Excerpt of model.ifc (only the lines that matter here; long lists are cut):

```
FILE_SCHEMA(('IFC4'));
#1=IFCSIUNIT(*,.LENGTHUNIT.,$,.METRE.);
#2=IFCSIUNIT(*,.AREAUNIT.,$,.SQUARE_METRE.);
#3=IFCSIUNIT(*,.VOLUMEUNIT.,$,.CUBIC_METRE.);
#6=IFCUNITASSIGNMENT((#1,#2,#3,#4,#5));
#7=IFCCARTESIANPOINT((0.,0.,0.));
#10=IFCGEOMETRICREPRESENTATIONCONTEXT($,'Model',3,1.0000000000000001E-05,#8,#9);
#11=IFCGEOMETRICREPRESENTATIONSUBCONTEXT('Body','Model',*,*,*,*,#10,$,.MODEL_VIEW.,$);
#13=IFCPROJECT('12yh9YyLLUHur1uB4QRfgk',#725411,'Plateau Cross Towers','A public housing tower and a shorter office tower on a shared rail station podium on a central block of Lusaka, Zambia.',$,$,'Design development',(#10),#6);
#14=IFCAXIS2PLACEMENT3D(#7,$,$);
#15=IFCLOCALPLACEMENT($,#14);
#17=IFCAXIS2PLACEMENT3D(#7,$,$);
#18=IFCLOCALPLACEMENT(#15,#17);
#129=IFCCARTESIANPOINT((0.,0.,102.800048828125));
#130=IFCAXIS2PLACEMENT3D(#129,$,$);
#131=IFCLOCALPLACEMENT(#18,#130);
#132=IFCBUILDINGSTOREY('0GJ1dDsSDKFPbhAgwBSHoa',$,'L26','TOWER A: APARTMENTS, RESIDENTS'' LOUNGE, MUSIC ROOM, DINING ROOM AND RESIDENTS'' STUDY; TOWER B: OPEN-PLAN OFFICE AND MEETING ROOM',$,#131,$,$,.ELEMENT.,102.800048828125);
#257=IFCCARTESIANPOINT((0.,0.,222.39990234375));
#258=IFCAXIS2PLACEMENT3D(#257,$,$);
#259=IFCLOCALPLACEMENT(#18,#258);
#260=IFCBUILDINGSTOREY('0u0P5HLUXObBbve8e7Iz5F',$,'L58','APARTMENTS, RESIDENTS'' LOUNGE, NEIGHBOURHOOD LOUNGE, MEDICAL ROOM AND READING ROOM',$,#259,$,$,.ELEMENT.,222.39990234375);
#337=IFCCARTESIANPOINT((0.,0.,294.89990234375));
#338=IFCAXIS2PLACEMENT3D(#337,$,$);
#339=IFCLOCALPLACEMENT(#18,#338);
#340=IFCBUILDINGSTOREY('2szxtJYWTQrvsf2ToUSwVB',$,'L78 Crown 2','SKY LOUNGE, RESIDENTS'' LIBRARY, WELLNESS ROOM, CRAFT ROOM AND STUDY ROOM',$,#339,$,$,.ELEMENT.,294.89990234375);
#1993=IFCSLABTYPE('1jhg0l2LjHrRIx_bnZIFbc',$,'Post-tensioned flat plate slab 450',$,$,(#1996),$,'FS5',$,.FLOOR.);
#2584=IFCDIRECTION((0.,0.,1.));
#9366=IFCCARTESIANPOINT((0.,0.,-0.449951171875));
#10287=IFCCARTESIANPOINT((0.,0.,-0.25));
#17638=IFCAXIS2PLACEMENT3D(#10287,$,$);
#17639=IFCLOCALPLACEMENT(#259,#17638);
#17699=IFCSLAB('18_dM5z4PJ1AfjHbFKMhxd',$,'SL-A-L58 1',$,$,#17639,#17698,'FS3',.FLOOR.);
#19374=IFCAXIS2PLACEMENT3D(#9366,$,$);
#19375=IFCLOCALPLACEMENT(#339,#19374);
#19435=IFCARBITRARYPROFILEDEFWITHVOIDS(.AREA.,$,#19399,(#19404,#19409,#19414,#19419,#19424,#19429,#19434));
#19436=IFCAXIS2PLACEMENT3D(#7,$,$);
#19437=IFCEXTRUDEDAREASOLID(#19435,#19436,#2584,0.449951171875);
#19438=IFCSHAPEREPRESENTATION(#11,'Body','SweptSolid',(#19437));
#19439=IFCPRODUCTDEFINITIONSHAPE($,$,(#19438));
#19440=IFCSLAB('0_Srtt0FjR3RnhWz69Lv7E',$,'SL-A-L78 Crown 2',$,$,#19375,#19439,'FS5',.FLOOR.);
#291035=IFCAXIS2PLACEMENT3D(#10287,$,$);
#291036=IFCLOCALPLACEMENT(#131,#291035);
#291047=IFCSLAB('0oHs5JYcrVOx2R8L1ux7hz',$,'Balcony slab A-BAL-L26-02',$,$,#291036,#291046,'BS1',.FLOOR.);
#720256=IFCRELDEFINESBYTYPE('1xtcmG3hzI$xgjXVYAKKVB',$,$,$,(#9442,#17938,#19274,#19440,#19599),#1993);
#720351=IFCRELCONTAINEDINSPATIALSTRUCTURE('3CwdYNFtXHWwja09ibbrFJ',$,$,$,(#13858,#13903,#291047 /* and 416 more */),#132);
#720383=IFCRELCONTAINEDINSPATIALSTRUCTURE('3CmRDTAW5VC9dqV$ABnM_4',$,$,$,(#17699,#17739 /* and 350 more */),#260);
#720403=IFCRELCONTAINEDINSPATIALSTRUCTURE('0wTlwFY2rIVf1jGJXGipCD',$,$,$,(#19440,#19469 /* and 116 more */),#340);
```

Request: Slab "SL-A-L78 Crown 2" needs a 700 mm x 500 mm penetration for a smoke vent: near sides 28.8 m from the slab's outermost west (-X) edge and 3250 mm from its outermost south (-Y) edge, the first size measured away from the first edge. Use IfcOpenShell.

```python
import numpy as np
import ifcopenshell
import ifcopenshell.api.feature
import ifcopenshell.api.geometry
import ifcopenshell.api.root
import ifcopenshell.geom
import ifcopenshell.util.placement
import ifcopenshell.util.representation
import ifcopenshell.util.shape
import ifcopenshell.util.unit

model = ifcopenshell.open("model.ifc")
unit_scale = ifcopenshell.util.unit.calculate_unit_scale(model)
settings = ifcopenshell.geom.settings()


def volume(element):
    """Net volume in cubic metres, openings subtracted."""
    shape = ifcopenshell.geom.create_shape(settings, element)
    return ifcopenshell.util.shape.get_volume(shape.geometry)


slab = model.by_guid("0_Srtt0FjR3RnhWz69Lv7E")
before = volume(slab)

# Extent in the slab's own axes, in metres. The edges named are its -X and -Y sides.
slab_shape = ifcopenshell.geom.create_shape(settings, slab)
vertices = ifcopenshell.util.shape.get_vertices(slab_shape.geometry)
x_min, y_min, bottom = vertices.min(axis=0)
top = vertices[:, 2].max()

opening = ifcopenshell.api.root.create_entity(model, ifc_class="IfcOpeningElement", name="Smoke vent opening", predefined_type="OPENING")
context = ifcopenshell.util.representation.get_context(model, "Model", "Body", "MODEL_VIEW")
width, depth = 0.7, 0.5
outline = [(0.0, 0.0), (width, 0.0), (width, depth), (0.0, depth), (0.0, 0.0)]
# Overshoot both faces by 50 mm so the cut is clean.
shape = ifcopenshell.api.geometry.add_slab_representation(
    model, context=context, depth=top - bottom + 0.1, polyline=outline
)
ifcopenshell.api.geometry.assign_representation(model, product=opening, representation=shape)

matrix = ifcopenshell.util.placement.get_local_placement(slab.ObjectPlacement)
matrix[:, 3] = matrix @ np.append(np.array([x_min + 28.8, y_min + 3.25, bottom - 0.05]) / unit_scale, 1.0)
ifcopenshell.api.geometry.edit_object_placement(model, product=opening, matrix=matrix, is_si=False)
ifcopenshell.api.feature.add_feature(model, feature=opening, element=slab)

after = volume(slab)

print(f"slab volume {before:.3f} -> {after:.3f} m3")

model.write("model_rev.ifc")
```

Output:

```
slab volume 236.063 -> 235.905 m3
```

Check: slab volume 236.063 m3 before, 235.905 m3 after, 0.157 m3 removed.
